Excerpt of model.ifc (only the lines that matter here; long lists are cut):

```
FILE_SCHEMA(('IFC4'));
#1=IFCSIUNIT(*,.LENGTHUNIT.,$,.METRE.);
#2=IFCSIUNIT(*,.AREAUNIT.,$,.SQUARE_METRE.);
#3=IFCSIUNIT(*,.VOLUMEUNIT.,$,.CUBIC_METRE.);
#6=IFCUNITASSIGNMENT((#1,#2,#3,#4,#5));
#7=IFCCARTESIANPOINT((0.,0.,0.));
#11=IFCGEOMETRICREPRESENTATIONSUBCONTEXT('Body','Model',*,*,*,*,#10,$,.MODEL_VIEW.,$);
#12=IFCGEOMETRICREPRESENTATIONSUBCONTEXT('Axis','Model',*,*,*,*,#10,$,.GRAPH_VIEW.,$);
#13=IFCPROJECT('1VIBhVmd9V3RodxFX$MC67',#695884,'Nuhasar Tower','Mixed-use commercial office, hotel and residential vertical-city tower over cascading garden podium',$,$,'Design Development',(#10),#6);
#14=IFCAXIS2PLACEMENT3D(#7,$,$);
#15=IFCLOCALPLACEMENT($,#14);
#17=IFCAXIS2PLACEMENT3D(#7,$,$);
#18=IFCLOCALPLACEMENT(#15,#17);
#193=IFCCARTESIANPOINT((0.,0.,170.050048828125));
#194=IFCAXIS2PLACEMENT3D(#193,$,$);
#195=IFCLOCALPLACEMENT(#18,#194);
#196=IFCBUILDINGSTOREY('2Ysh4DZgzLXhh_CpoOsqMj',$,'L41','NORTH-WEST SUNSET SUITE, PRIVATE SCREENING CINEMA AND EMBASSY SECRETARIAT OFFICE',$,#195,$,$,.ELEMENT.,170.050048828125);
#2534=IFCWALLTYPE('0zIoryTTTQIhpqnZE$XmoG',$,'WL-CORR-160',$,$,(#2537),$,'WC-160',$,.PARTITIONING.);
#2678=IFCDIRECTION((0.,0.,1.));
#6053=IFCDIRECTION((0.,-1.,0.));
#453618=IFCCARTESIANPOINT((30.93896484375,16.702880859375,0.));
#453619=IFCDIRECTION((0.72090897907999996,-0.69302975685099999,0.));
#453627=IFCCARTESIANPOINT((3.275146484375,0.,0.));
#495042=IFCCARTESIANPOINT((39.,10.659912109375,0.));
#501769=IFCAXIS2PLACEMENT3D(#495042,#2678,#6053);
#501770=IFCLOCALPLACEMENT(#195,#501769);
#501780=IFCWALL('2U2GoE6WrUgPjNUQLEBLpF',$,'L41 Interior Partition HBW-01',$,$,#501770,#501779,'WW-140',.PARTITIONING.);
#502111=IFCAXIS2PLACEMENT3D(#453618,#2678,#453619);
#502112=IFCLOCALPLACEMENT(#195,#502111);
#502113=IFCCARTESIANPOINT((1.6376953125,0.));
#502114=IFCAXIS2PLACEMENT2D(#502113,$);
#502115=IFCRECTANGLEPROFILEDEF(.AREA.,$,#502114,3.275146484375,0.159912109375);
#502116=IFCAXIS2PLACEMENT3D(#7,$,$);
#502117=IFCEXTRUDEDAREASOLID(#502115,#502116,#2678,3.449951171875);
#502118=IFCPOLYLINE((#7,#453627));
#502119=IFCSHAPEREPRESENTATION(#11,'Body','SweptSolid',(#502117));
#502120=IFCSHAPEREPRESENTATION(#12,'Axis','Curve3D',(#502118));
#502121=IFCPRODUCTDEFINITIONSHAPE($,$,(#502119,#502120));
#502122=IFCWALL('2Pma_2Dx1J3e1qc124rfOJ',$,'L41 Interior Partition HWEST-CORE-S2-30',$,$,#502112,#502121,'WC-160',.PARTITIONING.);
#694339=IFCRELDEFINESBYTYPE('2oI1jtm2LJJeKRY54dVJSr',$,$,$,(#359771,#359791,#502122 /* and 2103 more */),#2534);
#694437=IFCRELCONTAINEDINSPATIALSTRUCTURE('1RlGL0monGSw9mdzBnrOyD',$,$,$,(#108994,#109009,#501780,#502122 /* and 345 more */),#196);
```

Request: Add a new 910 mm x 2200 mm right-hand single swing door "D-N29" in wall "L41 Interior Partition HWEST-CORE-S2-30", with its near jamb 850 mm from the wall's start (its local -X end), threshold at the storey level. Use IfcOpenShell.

```python
import numpy as np
import ifcopenshell
import ifcopenshell.api.feature
import ifcopenshell.api.geometry
import ifcopenshell.api.root
import ifcopenshell.api.spatial
import ifcopenshell.geom
import ifcopenshell.util.element
import ifcopenshell.util.placement
import ifcopenshell.util.representation
import ifcopenshell.util.shape
import ifcopenshell.util.unit

model = ifcopenshell.open("model.ifc")
unit_scale = ifcopenshell.util.unit.calculate_unit_scale(model)
settings = ifcopenshell.geom.settings()


def volume(element):
    """Net volume in cubic metres, openings subtracted."""
    shape = ifcopenshell.geom.create_shape(settings, element)
    return ifcopenshell.util.shape.get_volume(shape.geometry)


wall = model.by_guid("2Pma_2Dx1J3e1qc124rfOJ")
storey = ifcopenshell.util.element.get_container(wall, ifc_class="IfcBuildingStorey")
context = ifcopenshell.util.representation.get_context(model, "Model", "Body", "MODEL_VIEW")
before = volume(wall)

width, height, from_end, sill = 0.91, 2.2, 0.85, 0.0  # metres

# The wall runs along its own X axis, and the end named is its -X end.
wall_shape = ifcopenshell.geom.create_shape(settings, wall)
x, y, z = ifcopenshell.util.shape.get_vertices(wall_shape.geometry).T
start = x.min() + from_end
face, thickness = float(y.min()), float(y.max() - y.min())
wall_matrix = ifcopenshell.util.placement.get_local_placement(wall.ObjectPlacement)
level = ifcopenshell.util.placement.get_local_placement(storey.ObjectPlacement)[2, 3]


def in_wall(x, y):
    """Placement at x, y metres in the wall's axes, at sill height."""
    matrix = wall_matrix.copy()
    matrix[:, 3] = wall_matrix @ np.array([x / unit_scale, y / unit_scale, 0.0, 1.0])
    matrix[2, 3] = level + sill / unit_scale
    return matrix


# Opening: a box that overshoots both wall faces by 50 mm.
opening = ifcopenshell.api.root.create_entity(model, ifc_class="IfcOpeningElement", predefined_type="OPENING")
box = ifcopenshell.api.geometry.add_wall_representation(
    model, context=context, length=width, height=height, thickness=thickness + 0.1
)
ifcopenshell.api.geometry.assign_representation(model, product=opening, representation=box)
ifcopenshell.api.geometry.edit_object_placement(model, product=opening, matrix=in_wall(start, face - 0.05), is_si=False)
ifcopenshell.api.feature.add_feature(model, feature=opening, element=wall)

door = ifcopenshell.api.root.create_entity(model, ifc_class="IfcDoor", name="D-N29", predefined_type="DOOR")
door.OverallWidth, door.OverallHeight = width / unit_scale, height / unit_scale
door.OperationType = "SINGLE_SWING_RIGHT"
body = ifcopenshell.api.geometry.add_door_representation(
    model,
    context=context,
    overall_width=door.OverallWidth,
    overall_height=door.OverallHeight,
    operation_type="SINGLE_SWING_RIGHT",
    lining_properties={"LiningDepth": thickness / unit_scale, "ThresholdDepth": thickness / unit_scale},
)
ifcopenshell.api.geometry.assign_representation(model, product=door, representation=body)
ifcopenshell.api.spatial.assign_container(model, products=[door], relating_structure=storey)
ifcopenshell.api.feature.add_filling(model, opening=opening, element=door)

# The lining spans the wall, so the door starts at the wall face.
ifcopenshell.api.geometry.edit_object_placement(model, product=door, matrix=in_wall(start, face), is_si=False)

after = volume(wall)

print(f"wall volume {before:.3f} -> {after:.3f} m3")

model.write("model-out.ifc")
```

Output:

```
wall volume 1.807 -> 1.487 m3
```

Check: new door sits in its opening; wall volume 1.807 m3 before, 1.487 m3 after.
